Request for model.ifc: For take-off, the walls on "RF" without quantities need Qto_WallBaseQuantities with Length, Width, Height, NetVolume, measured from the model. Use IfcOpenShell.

First a look at what the model holds.

```python
import ifcopenshell
import ifcopenshell.util.element
import ifcopenshell.util.unit

model = ifcopenshell.open("model.ifc")
print(model.schema)
for unit_type in ("LENGTHUNIT", "AREAUNIT", "VOLUMEUNIT"):
    print(unit_type, ifcopenshell.util.unit.calculate_unit_scale(model, unit_type))
storey = next(s for s in model.by_type("IfcBuildingStorey") if s.Name == "RF")
walls = [e for e in ifcopenshell.util.element.get_decomposition(storey) if e.is_a("IfcWall")]
for e in sorted(walls, key=lambda e: e.id()):
    print(e.id(), e.is_a(), e.Name, list(ifcopenshell.util.element.get_psets(e, qtos_only=True)), sep=" | ")
```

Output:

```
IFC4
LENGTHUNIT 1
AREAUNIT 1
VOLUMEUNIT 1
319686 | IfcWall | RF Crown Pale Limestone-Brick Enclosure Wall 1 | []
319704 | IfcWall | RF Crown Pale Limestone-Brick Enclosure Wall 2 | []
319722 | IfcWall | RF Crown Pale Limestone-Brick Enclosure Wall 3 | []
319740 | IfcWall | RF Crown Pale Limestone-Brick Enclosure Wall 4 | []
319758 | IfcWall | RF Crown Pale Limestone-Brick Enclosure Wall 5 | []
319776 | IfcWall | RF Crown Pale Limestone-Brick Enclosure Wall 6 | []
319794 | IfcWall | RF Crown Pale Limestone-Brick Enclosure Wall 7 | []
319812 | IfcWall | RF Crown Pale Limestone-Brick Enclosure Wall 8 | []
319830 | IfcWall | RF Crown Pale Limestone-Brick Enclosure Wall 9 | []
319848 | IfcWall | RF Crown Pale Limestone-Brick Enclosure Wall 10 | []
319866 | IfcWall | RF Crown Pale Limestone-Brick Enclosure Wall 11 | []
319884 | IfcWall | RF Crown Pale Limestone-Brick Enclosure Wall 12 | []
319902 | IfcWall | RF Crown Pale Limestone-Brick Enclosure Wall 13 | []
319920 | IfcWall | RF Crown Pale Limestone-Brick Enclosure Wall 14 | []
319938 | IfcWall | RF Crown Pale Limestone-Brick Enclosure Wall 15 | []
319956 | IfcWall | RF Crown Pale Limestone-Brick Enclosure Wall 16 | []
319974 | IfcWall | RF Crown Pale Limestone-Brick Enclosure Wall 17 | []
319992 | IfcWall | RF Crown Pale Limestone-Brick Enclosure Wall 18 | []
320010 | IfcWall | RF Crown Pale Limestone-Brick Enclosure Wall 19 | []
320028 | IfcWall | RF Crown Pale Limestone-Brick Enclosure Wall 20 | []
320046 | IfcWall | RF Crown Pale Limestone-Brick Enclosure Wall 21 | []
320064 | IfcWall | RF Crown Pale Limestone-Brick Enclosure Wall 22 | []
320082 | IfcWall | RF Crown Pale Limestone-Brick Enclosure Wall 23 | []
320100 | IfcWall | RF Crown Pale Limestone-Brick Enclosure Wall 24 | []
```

```python
import ifcopenshell
import ifcopenshell.api.pset
import ifcopenshell.geom
import ifcopenshell.util.element
import ifcopenshell.util.shape
import ifcopenshell.util.unit

model = ifcopenshell.open("model.ifc")
unit_scale = ifcopenshell.util.unit.calculate_unit_scale(model)
volume_scale = ifcopenshell.util.unit.calculate_unit_scale(model, "VOLUMEUNIT")
settings = ifcopenshell.geom.settings()

storey = next(s for s in model.by_type("IfcBuildingStorey") if s.Name == "RF")
walls = [e for e in ifcopenshell.util.element.get_decomposition(storey) if e.is_a("IfcWall")]

for e in sorted(walls, key=lambda e: e.id()):
    if ifcopenshell.util.element.get_psets(e, qtos_only=True, should_inherit=False):
        continue
    # Geometry comes back in metres, in the element's own axes.
    shape = ifcopenshell.geom.create_shape(settings, e)
    values = {
        "Length": ifcopenshell.util.shape.get_x(shape.geometry) / unit_scale,
        "Width": ifcopenshell.util.shape.get_y(shape.geometry) / unit_scale,
        "Height": ifcopenshell.util.shape.get_z(shape.geometry) / unit_scale,
        "NetVolume": ifcopenshell.util.shape.get_volume(shape.geometry) / volume_scale,
    }
    qto = ifcopenshell.api.pset.add_qto(model, product=e, name="Qto_WallBaseQuantities")
    ifcopenshell.api.pset.edit_qto(model, qto=qto, properties=values)
    print(e.id(), {k: round(v, 3) for k, v in values.items()})

model.write("model_v2.ifc")
```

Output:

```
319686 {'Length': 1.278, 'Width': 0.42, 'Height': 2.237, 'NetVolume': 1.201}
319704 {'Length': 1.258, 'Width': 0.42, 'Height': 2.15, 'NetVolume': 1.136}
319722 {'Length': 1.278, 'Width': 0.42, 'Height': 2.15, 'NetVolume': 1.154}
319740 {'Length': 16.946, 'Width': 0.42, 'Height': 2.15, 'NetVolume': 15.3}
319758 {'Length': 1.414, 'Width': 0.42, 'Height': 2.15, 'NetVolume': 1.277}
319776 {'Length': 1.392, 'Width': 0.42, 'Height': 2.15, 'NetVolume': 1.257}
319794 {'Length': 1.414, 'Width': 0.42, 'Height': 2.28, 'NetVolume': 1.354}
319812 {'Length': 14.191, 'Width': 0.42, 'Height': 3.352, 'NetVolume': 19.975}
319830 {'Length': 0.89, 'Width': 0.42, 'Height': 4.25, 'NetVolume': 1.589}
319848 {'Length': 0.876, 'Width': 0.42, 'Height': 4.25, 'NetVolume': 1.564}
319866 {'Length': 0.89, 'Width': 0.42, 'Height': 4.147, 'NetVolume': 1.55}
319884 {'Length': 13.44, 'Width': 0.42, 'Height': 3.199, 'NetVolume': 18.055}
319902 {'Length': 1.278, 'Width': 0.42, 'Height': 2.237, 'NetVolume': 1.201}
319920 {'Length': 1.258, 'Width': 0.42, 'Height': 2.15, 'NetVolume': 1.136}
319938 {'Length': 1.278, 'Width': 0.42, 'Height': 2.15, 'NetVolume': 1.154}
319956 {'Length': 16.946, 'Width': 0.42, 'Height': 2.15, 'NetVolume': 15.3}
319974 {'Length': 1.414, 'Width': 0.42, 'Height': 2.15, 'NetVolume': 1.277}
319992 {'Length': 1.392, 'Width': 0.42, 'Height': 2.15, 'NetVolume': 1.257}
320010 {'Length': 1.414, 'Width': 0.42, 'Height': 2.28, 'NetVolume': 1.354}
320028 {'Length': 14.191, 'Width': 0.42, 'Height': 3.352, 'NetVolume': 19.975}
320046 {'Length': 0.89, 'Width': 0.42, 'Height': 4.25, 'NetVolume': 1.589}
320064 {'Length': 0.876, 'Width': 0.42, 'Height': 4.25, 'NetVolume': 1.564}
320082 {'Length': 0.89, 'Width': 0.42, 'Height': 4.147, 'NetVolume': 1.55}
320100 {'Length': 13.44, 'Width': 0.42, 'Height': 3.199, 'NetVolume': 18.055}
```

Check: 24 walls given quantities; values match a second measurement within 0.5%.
